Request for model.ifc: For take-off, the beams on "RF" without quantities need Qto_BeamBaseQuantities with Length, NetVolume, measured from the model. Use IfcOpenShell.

First a look at what the model holds.

```python
import ifcopenshell
import ifcopenshell.util.element
import ifcopenshell.util.unit

model = ifcopenshell.open("model.ifc")
print(model.schema)
for unit_type in ("LENGTHUNIT", "AREAUNIT", "VOLUMEUNIT"):
    print(unit_type, ifcopenshell.util.unit.calculate_unit_scale(model, unit_type))
storey = next(s for s in model.by_type("IfcBuildingStorey") if s.Name == "RF")
beams = [e for e in ifcopenshell.util.element.get_decomposition(storey) if e.is_a("IfcBeam")]
for e in sorted(beams, key=lambda e: e.id()):
    print(e.id(), e.is_a(), e.Name, list(ifcopenshell.util.element.get_psets(e, qtos_only=True)), sep=" | ")
```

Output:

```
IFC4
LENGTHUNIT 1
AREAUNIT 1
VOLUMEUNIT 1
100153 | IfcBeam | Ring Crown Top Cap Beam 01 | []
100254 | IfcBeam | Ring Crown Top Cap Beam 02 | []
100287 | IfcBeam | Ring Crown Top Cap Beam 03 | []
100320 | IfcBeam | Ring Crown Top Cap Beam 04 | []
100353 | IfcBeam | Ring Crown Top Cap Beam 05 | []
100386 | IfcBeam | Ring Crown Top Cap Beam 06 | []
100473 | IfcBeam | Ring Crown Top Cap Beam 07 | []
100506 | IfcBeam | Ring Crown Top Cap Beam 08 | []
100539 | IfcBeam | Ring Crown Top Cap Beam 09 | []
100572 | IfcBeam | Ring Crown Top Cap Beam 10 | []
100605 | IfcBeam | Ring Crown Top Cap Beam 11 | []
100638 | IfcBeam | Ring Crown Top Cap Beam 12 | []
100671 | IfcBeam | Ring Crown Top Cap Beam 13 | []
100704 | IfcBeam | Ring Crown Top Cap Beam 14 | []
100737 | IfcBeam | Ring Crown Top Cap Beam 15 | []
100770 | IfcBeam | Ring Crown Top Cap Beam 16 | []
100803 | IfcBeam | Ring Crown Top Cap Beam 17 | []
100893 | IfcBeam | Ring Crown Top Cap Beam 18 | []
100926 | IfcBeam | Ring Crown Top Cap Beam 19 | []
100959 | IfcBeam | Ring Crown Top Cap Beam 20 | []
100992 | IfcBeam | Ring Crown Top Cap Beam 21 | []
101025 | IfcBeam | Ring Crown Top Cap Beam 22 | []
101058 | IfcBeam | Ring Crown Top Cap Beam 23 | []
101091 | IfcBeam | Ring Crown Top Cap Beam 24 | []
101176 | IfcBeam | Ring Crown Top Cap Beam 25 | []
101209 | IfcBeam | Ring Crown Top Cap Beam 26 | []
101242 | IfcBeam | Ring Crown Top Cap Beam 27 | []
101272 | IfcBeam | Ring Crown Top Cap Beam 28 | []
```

```python
import ifcopenshell
import ifcopenshell.api.pset
import ifcopenshell.geom
import ifcopenshell.util.element
import ifcopenshell.util.shape
import ifcopenshell.util.unit

model = ifcopenshell.open("model.ifc")
unit_scale = ifcopenshell.util.unit.calculate_unit_scale(model)
volume_scale = ifcopenshell.util.unit.calculate_unit_scale(model, "VOLUMEUNIT")
settings = ifcopenshell.geom.settings()

storey = next(s for s in model.by_type("IfcBuildingStorey") if s.Name == "RF")
beams = [e for e in ifcopenshell.util.element.get_decomposition(storey) if e.is_a("IfcBeam")]

for e in sorted(beams, key=lambda e: e.id()):
    if ifcopenshell.util.element.get_psets(e, qtos_only=True, should_inherit=False):
        continue
    # Geometry comes back in metres, in the element's own axes.
    shape = ifcopenshell.geom.create_shape(settings, e)
    values = {
        "Length": ifcopenshell.util.shape.get_max_xyz(shape.geometry) / unit_scale,
        "NetVolume": ifcopenshell.util.shape.get_volume(shape.geometry) / volume_scale,
    }
    qto = ifcopenshell.api.pset.add_qto(model, product=e, name="Qto_BeamBaseQuantities")
    ifcopenshell.api.pset.edit_qto(model, qto=qto, properties=values)
    print(e.id(), {k: round(v, 3) for k, v in values.items()})

model.write("model-out.ifc")
```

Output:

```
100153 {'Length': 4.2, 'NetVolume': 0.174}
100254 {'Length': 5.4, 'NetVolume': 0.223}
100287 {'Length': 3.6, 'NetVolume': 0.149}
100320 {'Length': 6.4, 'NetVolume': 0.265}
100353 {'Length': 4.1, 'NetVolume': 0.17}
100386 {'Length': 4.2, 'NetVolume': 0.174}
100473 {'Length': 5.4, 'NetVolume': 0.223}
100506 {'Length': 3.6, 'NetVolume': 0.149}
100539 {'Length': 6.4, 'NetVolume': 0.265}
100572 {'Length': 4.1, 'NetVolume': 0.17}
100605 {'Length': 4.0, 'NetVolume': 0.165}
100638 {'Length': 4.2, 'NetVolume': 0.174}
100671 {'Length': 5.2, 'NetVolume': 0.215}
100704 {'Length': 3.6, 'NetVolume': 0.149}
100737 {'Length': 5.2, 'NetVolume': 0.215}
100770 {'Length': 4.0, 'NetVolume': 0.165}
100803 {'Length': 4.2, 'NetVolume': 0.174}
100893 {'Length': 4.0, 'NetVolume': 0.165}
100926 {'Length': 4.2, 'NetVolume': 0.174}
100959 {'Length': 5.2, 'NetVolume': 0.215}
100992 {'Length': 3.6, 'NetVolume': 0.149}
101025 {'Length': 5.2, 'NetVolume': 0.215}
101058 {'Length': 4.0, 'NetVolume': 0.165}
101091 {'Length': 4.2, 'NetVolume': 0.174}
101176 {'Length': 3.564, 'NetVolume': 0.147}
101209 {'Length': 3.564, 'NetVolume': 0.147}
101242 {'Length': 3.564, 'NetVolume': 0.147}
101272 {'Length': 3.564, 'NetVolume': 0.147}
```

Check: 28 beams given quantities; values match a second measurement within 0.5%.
